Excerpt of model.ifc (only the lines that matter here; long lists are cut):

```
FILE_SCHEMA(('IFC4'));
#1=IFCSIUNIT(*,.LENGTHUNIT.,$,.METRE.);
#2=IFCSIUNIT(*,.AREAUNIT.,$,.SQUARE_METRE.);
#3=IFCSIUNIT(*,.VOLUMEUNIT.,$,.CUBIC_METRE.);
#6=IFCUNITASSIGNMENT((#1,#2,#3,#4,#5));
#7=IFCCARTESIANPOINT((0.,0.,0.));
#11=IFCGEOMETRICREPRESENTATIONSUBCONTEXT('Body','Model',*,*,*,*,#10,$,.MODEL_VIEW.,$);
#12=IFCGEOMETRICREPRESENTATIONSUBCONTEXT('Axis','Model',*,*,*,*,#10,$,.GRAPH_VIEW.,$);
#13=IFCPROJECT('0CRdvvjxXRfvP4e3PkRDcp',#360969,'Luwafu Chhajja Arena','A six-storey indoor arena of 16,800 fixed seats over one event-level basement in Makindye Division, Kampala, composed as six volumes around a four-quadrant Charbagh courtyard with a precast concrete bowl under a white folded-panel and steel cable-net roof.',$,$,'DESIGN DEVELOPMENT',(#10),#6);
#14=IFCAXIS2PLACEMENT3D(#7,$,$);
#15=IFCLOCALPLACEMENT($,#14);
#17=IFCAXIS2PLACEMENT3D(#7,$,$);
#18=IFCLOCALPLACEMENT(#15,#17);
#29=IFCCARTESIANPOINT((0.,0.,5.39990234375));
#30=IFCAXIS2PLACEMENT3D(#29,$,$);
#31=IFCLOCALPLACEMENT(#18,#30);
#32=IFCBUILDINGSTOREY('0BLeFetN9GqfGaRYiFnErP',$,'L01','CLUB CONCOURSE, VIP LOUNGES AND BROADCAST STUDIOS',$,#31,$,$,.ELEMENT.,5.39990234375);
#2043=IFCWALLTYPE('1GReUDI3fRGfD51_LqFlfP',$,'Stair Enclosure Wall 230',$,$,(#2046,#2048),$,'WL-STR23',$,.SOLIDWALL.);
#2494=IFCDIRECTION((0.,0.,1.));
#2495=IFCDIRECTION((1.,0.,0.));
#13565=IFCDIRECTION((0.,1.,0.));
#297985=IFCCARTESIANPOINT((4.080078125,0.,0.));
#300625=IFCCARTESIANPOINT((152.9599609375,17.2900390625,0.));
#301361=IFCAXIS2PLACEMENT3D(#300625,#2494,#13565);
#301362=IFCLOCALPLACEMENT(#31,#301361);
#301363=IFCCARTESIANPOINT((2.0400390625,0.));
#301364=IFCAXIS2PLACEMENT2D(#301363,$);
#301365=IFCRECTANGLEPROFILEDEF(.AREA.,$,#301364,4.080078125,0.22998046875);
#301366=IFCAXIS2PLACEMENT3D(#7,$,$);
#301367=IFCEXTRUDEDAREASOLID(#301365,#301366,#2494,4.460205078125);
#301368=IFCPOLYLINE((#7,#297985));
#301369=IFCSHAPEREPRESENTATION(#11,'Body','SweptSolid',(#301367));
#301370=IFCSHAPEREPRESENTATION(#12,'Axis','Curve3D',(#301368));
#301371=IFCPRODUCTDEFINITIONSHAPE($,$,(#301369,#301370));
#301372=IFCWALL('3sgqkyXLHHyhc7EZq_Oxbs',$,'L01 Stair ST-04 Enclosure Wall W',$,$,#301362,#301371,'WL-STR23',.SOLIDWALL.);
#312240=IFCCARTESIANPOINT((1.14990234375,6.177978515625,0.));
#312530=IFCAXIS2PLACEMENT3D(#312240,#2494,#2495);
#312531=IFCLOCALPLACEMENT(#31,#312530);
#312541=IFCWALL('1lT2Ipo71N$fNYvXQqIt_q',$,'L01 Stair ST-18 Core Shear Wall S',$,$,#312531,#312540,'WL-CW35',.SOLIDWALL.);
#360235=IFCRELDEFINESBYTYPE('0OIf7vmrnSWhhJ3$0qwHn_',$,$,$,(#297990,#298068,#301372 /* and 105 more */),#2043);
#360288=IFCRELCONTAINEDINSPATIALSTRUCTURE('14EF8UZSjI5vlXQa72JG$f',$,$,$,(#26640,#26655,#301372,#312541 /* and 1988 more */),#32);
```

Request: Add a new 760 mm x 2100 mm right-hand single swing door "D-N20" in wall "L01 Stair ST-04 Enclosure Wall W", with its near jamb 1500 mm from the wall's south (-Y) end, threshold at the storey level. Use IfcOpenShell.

```python
import numpy as np
import ifcopenshell
import ifcopenshell.api.feature
import ifcopenshell.api.geometry
import ifcopenshell.api.root
import ifcopenshell.api.spatial
import ifcopenshell.geom
import ifcopenshell.util.element
import ifcopenshell.util.placement
import ifcopenshell.util.representation
import ifcopenshell.util.shape
import ifcopenshell.util.unit

model = ifcopenshell.open("model.ifc")
unit_scale = ifcopenshell.util.unit.calculate_unit_scale(model)
settings = ifcopenshell.geom.settings()


def volume(element):
    """Net volume in cubic metres, openings subtracted."""
    shape = ifcopenshell.geom.create_shape(settings, element)
    return ifcopenshell.util.shape.get_volume(shape.geometry)


wall = model.by_guid("3sgqkyXLHHyhc7EZq_Oxbs")
storey = ifcopenshell.util.element.get_container(wall, ifc_class="IfcBuildingStorey")
context = ifcopenshell.util.representation.get_context(model, "Model", "Body", "MODEL_VIEW")
before = volume(wall)

width, height, from_end, sill = 0.76, 2.1, 1.5, 0.0  # metres

# The wall runs along its own X axis, and the end named is its -X end.
wall_shape = ifcopenshell.geom.create_shape(settings, wall)
x, y, z = ifcopenshell.util.shape.get_vertices(wall_shape.geometry).T
start = x.min() + from_end
face, thickness = float(y.min()), float(y.max() - y.min())
wall_matrix = ifcopenshell.util.placement.get_local_placement(wall.ObjectPlacement)
level = ifcopenshell.util.placement.get_local_placement(storey.ObjectPlacement)[2, 3]


def in_wall(x, y):
    """Placement at x, y metres in the wall's axes, at sill height."""
    matrix = wall_matrix.copy()
    matrix[:, 3] = wall_matrix @ np.array([x / unit_scale, y / unit_scale, 0.0, 1.0])
    matrix[2, 3] = level + sill / unit_scale
    return matrix


# Opening: a box that overshoots both wall faces by 50 mm.
opening = ifcopenshell.api.root.create_entity(model, ifc_class="IfcOpeningElement", predefined_type="OPENING")
box = ifcopenshell.api.geometry.add_wall_representation(
    model, context=context, length=width, height=height, thickness=thickness + 0.1
)
ifcopenshell.api.geometry.assign_representation(model, product=opening, representation=box)
ifcopenshell.api.geometry.edit_object_placement(model, product=opening, matrix=in_wall(start, face - 0.05), is_si=False)
ifcopenshell.api.feature.add_feature(model, feature=opening, element=wall)

door = ifcopenshell.api.root.create_entity(model, ifc_class="IfcDoor", name="D-N20", predefined_type="DOOR")
door.OverallWidth, door.OverallHeight = width / unit_scale, height / unit_scale
door.OperationType = "SINGLE_SWING_RIGHT"
body = ifcopenshell.api.geometry.add_door_representation(
    model,
    context=context,
    overall_width=door.OverallWidth,
    overall_height=door.OverallHeight,
    operation_type="SINGLE_SWING_RIGHT",
    lining_properties={"LiningDepth": thickness / unit_scale, "ThresholdDepth": thickness / unit_scale},
)
ifcopenshell.api.geometry.assign_representation(model, product=door, representation=body)
ifcopenshell.api.spatial.assign_container(model, products=[door], relating_structure=storey)
ifcopenshell.api.feature.add_filling(model, opening=opening, element=door)

# The lining spans the wall, so the door starts at the wall face.
ifcopenshell.api.geometry.edit_object_placement(model, product=door, matrix=in_wall(start, face), is_si=False)

after = volume(wall)

print(f"wall volume {before:.3f} -> {after:.3f} m3")

model.write("model_v2.ifc")
```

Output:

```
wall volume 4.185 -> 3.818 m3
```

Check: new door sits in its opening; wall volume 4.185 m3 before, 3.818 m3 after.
